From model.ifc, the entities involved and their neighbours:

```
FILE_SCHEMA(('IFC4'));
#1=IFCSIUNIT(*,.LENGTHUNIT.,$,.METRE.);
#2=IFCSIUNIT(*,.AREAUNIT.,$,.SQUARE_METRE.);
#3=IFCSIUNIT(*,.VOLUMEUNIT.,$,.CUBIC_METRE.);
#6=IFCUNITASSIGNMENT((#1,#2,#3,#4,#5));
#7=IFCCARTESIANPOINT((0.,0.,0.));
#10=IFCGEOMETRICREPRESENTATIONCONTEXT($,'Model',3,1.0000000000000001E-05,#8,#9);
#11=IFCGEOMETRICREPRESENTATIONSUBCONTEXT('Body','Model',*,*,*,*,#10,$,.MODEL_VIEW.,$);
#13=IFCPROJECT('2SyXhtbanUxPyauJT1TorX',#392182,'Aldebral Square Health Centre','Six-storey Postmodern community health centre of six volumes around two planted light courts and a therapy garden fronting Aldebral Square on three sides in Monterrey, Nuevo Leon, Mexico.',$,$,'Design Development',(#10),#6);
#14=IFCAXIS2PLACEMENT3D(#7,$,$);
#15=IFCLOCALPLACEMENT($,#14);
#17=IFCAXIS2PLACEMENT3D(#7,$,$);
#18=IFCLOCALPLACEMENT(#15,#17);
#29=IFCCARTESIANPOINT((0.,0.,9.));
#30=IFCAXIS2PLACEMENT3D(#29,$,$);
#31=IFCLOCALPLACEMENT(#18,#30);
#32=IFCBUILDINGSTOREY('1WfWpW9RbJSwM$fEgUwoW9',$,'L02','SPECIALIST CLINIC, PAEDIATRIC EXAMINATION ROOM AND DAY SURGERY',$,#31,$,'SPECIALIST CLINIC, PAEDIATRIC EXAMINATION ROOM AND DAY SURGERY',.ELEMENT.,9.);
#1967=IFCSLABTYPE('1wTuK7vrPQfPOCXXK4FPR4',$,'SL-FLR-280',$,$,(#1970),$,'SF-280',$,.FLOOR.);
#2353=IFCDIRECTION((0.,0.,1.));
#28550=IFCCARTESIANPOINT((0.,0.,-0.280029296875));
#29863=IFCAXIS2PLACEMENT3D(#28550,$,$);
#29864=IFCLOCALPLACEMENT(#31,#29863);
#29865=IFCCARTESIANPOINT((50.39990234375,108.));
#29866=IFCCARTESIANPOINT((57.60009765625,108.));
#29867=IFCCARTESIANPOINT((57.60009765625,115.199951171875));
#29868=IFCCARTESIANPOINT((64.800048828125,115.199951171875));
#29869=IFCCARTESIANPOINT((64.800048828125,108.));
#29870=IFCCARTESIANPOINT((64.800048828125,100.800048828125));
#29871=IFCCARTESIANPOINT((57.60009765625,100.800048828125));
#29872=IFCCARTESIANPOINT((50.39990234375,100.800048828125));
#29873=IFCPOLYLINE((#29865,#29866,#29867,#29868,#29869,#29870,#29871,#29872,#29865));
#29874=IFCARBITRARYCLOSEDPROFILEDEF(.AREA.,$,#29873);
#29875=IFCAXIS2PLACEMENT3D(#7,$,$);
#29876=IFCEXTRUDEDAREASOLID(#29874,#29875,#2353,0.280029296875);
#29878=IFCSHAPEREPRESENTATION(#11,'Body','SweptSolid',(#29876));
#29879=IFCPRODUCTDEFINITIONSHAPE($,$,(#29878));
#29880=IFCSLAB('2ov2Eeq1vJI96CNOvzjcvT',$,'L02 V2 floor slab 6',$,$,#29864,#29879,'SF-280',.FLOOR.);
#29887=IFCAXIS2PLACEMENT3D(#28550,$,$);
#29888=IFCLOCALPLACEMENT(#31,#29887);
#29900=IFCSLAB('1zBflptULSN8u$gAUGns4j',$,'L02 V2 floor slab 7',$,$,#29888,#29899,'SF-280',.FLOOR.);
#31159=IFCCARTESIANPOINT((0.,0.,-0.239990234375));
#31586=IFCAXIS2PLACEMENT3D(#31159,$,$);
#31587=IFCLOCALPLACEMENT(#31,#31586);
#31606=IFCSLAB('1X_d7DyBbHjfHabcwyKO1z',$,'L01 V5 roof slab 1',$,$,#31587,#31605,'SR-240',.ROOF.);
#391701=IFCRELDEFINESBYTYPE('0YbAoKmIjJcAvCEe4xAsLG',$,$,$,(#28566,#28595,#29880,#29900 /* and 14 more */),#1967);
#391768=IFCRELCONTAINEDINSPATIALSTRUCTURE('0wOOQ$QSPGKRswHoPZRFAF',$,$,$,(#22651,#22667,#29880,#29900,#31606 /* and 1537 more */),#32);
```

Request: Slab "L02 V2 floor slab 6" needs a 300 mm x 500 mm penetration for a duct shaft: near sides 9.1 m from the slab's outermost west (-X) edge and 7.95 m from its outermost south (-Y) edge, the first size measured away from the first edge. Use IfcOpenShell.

```python
import numpy as np
import ifcopenshell
import ifcopenshell.api.feature
import ifcopenshell.api.geometry
import ifcopenshell.api.root
import ifcopenshell.geom
import ifcopenshell.util.placement
import ifcopenshell.util.representation
import ifcopenshell.util.shape
import ifcopenshell.util.unit

model = ifcopenshell.open("model.ifc")
unit_scale = ifcopenshell.util.unit.calculate_unit_scale(model)
settings = ifcopenshell.geom.settings()


def volume(element):
    """Net volume in cubic metres, openings subtracted."""
    shape = ifcopenshell.geom.create_shape(settings, element)
    return ifcopenshell.util.shape.get_volume(shape.geometry)


slab = model.by_guid("2ov2Eeq1vJI96CNOvzjcvT")
before = volume(slab)

# Extent in the slab's own axes, in metres. The edges named are its -X and -Y sides.
slab_shape = ifcopenshell.geom.create_shape(settings, slab)
vertices = ifcopenshell.util.shape.get_vertices(slab_shape.geometry)
x_min, y_min, bottom = vertices.min(axis=0)
top = vertices[:, 2].max()

opening = ifcopenshell.api.root.create_entity(model, ifc_class="IfcOpeningElement", name="Duct shaft opening", predefined_type="OPENING")
context = ifcopenshell.util.representation.get_context(model, "Model", "Body", "MODEL_VIEW")
width, depth = 0.3, 0.5
outline = [(0.0, 0.0), (width, 0.0), (width, depth), (0.0, depth), (0.0, 0.0)]
# Overshoot both faces by 50 mm so the cut is clean.
shape = ifcopenshell.api.geometry.add_slab_representation(
    model, context=context, depth=top - bottom + 0.1, polyline=outline
)
ifcopenshell.api.geometry.assign_representation(model, product=opening, representation=shape)

matrix = ifcopenshell.util.placement.get_local_placement(slab.ObjectPlacement)
matrix[:, 3] = matrix @ np.append(np.array([x_min + 9.1, y_min + 7.95, bottom - 0.05]) / unit_scale, 1.0)
ifcopenshell.api.geometry.edit_object_placement(model, product=opening, matrix=matrix, is_si=False)
ifcopenshell.api.feature.add_feature(model, feature=opening, element=slab)

after = volume(slab)

print(f"slab volume {before:.3f} -> {after:.3f} m3")

model.write("model_updated.ifc")
```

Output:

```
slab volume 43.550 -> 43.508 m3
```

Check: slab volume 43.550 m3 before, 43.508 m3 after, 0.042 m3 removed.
